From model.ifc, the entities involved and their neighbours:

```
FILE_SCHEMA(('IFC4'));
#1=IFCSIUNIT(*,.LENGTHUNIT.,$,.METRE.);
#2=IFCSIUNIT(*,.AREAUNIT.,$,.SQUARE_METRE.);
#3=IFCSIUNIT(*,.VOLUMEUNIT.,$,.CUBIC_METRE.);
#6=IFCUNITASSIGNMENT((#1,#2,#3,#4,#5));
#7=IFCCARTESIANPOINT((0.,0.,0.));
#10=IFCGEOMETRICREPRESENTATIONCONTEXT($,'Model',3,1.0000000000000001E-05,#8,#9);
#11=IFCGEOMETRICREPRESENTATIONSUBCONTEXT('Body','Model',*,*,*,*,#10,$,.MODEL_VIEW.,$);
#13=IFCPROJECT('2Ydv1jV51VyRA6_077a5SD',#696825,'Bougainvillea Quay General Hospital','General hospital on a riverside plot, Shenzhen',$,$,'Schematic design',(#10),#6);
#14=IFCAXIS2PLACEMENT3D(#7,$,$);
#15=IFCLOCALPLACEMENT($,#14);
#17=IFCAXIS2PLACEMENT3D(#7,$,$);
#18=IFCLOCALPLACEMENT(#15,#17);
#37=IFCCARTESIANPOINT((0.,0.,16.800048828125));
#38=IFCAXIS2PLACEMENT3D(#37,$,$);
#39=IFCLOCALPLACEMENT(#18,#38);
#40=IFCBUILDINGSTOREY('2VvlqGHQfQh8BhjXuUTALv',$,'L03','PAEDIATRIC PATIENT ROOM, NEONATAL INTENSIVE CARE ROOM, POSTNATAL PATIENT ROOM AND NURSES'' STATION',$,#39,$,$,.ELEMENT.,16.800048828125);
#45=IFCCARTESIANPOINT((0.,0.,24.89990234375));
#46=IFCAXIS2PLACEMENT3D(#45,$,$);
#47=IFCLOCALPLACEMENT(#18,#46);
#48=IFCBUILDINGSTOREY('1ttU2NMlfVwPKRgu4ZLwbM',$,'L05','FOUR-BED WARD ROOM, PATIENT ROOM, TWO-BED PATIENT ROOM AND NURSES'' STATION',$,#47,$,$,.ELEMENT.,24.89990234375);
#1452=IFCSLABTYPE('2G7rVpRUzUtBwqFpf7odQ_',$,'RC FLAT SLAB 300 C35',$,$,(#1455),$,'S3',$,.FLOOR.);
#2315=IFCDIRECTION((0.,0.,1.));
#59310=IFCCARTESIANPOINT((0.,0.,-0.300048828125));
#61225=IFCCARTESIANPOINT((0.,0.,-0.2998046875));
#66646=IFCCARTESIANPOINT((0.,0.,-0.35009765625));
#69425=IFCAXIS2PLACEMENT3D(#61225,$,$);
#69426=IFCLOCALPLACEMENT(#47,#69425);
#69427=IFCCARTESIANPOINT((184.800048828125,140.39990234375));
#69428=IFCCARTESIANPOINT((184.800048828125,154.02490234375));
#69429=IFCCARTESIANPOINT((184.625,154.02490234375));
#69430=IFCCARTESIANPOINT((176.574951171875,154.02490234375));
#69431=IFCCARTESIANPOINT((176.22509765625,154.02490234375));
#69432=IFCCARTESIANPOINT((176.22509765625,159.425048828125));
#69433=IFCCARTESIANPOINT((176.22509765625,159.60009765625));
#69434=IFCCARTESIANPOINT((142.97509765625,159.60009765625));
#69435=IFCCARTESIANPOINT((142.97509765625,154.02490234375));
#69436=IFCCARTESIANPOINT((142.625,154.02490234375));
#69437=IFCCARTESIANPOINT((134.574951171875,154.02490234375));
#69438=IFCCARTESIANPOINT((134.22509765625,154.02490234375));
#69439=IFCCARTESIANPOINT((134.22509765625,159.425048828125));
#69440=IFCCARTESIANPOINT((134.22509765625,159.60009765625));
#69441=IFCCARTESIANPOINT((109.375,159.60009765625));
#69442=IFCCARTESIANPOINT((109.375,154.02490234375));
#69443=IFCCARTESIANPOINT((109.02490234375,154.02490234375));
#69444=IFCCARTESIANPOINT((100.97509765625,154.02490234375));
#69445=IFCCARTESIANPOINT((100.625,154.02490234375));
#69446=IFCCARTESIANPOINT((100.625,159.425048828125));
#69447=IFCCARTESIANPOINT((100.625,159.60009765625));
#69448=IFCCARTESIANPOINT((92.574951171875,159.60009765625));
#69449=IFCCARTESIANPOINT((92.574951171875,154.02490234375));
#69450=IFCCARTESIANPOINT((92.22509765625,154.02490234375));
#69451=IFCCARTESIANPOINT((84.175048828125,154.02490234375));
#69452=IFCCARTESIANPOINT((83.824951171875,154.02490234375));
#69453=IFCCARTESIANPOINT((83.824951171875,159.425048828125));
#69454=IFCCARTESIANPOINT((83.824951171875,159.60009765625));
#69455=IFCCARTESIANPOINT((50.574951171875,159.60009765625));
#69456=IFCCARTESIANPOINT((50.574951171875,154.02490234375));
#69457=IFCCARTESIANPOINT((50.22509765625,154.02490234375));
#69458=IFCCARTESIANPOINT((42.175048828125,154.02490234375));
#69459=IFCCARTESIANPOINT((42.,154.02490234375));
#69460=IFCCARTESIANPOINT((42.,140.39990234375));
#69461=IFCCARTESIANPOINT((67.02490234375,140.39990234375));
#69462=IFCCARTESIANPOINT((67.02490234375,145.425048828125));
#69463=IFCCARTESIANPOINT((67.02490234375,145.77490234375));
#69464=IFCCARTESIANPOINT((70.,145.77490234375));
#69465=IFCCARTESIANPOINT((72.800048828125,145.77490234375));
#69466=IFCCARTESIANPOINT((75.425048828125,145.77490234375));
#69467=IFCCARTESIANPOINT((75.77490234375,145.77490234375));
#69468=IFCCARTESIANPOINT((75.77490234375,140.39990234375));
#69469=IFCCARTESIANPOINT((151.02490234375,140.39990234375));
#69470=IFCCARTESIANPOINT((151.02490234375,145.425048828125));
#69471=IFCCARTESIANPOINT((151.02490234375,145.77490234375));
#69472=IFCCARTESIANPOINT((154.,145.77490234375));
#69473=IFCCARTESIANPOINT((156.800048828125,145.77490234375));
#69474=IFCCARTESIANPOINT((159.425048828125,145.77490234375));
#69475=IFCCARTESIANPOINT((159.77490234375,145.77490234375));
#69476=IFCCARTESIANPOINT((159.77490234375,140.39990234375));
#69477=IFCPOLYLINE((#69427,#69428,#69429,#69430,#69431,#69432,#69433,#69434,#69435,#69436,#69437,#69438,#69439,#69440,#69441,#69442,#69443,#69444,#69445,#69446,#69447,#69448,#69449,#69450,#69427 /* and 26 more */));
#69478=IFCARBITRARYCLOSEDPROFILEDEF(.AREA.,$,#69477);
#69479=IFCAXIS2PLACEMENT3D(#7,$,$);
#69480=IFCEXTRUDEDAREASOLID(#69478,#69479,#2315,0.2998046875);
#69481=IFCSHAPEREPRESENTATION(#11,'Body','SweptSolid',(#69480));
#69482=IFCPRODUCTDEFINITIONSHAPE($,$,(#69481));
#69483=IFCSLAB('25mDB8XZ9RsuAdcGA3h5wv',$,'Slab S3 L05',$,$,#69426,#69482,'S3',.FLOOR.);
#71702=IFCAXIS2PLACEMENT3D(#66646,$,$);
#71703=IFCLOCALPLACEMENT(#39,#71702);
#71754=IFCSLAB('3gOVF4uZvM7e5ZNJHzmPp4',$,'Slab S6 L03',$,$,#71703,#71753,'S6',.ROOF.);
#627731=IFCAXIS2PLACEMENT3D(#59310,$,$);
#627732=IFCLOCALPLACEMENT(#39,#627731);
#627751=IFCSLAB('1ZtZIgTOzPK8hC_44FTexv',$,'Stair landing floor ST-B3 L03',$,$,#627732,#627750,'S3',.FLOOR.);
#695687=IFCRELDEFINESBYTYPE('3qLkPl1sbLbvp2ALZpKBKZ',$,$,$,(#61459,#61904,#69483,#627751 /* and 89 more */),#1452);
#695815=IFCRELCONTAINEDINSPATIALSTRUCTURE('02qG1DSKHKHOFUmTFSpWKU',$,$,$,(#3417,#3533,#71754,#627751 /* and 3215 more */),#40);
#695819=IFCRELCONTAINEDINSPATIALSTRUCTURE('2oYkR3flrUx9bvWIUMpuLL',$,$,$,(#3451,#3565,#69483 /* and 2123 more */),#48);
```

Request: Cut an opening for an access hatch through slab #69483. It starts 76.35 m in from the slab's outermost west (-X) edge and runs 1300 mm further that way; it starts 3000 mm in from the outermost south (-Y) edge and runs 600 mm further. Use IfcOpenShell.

```python
import numpy as np
import ifcopenshell
import ifcopenshell.api.feature
import ifcopenshell.api.geometry
import ifcopenshell.api.root
import ifcopenshell.geom
import ifcopenshell.util.placement
import ifcopenshell.util.representation
import ifcopenshell.util.shape
import ifcopenshell.util.unit

model = ifcopenshell.open("model.ifc")
unit_scale = ifcopenshell.util.unit.calculate_unit_scale(model)
settings = ifcopenshell.geom.settings()


def volume(element):
    """Net volume in cubic metres, openings subtracted."""
    shape = ifcopenshell.geom.create_shape(settings, element)
    return ifcopenshell.util.shape.get_volume(shape.geometry)


slab = model.by_guid("25mDB8XZ9RsuAdcGA3h5wv")
before = volume(slab)

# Extent in the slab's own axes, in metres. The edges named are its -X and -Y sides.
slab_shape = ifcopenshell.geom.create_shape(settings, slab)
vertices = ifcopenshell.util.shape.get_vertices(slab_shape.geometry)
x_min, y_min, bottom = vertices.min(axis=0)
top = vertices[:, 2].max()

opening = ifcopenshell.api.root.create_entity(model, ifc_class="IfcOpeningElement", name="Access hatch opening", predefined_type="OPENING")
context = ifcopenshell.util.representation.get_context(model, "Model", "Body", "MODEL_VIEW")
width, depth = 1.3, 0.6
outline = [(0.0, 0.0), (width, 0.0), (width, depth), (0.0, depth), (0.0, 0.0)]
# Overshoot both faces by 50 mm so the cut is clean.
shape = ifcopenshell.api.geometry.add_slab_representation(
    model, context=context, depth=top - bottom + 0.1, polyline=outline
)
ifcopenshell.api.geometry.assign_representation(model, product=opening, representation=shape)

matrix = ifcopenshell.util.placement.get_local_placement(slab.ObjectPlacement)
matrix[:, 3] = matrix @ np.append(np.array([x_min + 76.35, y_min + 3, bottom - 0.05]) / unit_scale, 1.0)
ifcopenshell.api.geometry.edit_object_placement(model, product=opening, matrix=matrix, is_si=False)
ifcopenshell.api.feature.add_feature(model, feature=opening, element=slab)

after = volume(slab)

print(f"slab volume {before:.3f} -> {after:.3f} m3")

model.write("model-out.ifc")
```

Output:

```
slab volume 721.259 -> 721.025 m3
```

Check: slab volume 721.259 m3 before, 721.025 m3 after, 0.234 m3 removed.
